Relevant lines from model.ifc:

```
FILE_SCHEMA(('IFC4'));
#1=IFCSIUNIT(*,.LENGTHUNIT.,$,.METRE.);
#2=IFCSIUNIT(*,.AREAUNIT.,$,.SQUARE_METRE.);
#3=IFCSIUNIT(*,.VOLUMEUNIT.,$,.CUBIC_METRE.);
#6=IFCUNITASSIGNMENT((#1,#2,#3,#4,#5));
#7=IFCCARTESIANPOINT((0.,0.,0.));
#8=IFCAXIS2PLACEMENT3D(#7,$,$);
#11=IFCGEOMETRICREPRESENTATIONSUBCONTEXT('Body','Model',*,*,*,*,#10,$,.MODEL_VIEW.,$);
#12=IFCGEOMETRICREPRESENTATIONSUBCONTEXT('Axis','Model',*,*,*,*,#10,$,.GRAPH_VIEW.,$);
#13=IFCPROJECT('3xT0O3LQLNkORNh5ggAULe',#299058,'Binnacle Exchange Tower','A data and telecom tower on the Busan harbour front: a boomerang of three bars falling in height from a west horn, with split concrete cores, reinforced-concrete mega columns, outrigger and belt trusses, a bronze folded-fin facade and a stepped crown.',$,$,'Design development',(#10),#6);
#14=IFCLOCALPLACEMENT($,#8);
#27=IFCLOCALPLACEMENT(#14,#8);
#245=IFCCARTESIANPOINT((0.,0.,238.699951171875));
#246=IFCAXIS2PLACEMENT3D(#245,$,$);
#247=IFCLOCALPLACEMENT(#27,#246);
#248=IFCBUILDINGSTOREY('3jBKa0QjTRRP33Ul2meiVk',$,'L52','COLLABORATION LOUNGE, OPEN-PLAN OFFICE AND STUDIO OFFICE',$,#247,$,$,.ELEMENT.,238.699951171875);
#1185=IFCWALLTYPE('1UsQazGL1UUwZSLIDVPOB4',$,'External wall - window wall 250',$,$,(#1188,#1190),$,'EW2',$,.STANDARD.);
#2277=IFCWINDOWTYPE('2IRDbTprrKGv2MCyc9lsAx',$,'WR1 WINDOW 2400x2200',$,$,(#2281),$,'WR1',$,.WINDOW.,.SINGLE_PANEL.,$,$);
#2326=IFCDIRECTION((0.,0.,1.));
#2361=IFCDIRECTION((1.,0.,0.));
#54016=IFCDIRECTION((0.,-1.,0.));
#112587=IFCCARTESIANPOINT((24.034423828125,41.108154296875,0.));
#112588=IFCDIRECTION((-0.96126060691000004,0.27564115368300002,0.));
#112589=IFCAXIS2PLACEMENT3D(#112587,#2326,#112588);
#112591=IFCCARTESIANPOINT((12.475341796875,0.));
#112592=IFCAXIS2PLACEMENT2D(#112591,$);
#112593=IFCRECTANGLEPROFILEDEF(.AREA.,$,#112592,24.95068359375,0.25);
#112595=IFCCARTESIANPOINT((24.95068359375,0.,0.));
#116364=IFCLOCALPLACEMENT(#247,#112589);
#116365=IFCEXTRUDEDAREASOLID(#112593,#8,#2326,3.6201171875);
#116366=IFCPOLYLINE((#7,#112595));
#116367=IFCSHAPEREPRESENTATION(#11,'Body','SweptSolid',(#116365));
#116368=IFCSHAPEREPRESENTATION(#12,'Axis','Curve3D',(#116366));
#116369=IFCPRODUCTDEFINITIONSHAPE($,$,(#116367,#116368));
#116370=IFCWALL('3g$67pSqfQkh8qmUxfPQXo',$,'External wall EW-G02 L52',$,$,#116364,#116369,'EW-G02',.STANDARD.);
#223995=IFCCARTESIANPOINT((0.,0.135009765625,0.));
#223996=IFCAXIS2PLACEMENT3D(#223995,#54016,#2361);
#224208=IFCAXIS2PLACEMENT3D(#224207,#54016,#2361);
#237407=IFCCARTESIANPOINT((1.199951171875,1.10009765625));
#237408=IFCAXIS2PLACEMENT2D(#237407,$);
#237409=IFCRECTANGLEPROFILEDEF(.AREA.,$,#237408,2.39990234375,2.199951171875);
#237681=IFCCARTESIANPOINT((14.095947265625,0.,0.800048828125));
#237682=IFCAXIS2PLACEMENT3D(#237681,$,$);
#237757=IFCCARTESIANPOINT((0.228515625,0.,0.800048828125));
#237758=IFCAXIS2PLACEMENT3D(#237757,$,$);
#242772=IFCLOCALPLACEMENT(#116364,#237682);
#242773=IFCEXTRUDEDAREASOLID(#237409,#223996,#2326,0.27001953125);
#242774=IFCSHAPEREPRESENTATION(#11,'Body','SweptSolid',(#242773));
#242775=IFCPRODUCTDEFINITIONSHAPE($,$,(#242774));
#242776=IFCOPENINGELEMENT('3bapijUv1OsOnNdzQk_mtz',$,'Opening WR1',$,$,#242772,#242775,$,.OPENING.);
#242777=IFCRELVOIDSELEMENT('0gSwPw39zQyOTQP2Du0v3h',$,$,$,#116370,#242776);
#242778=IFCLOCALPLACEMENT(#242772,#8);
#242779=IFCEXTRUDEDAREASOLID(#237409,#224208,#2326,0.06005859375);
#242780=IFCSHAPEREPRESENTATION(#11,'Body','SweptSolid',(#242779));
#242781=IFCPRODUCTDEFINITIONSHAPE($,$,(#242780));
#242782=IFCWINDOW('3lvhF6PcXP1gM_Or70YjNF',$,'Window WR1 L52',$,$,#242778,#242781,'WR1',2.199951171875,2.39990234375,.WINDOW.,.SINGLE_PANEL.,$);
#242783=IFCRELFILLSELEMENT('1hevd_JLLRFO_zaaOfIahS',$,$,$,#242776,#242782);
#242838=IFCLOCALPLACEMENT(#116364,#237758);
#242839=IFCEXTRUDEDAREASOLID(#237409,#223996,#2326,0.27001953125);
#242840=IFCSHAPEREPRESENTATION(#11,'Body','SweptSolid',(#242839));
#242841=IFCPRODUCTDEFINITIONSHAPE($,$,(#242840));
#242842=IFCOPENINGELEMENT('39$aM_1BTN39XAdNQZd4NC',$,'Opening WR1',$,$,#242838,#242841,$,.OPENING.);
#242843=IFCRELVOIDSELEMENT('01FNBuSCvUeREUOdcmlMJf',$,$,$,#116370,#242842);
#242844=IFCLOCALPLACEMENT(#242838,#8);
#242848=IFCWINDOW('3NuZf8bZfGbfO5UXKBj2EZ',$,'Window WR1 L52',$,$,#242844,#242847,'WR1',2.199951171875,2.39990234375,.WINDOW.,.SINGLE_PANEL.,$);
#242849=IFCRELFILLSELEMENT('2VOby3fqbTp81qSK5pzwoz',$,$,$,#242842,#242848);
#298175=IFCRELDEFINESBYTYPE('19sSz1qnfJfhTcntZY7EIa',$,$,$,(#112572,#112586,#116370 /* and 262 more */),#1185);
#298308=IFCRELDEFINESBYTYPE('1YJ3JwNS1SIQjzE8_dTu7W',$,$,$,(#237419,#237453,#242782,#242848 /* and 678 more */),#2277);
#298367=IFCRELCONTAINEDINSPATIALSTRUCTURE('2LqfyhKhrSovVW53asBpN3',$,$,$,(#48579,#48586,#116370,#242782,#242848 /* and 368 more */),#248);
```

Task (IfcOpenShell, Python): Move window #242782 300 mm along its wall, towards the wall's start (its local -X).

```python
import ifcopenshell
import ifcopenshell.api.geometry
import ifcopenshell.util.placement

model = ifcopenshell.open("model.ifc")

window = model.by_guid("3lvhF6PcXP1gM_Or70YjNF")
opening = window.FillsVoids[0].RelatingOpeningElement
wall = opening.VoidsElements[0].RelatingBuildingElement

wall_matrix = ifcopenshell.util.placement.get_local_placement(wall.ObjectPlacement)
shift = wall_matrix[:3, 0] * -0.3
before = ifcopenshell.util.placement.get_local_placement(window.ObjectPlacement)[:3, 3].copy()

# The window is placed relative to its opening, so it follows when the opening moves.
matrix = ifcopenshell.util.placement.get_local_placement(opening.ObjectPlacement)
matrix[:3, 3] += shift
ifcopenshell.api.geometry.edit_object_placement(
    model, product=opening, matrix=matrix, is_si=False, should_transform_children=True
)

after = ifcopenshell.util.placement.get_local_placement(window.ObjectPlacement)[:3, 3]
print("window moved by", (after - before).round(3) + 0.0)

model.write("model-out.ifc")
```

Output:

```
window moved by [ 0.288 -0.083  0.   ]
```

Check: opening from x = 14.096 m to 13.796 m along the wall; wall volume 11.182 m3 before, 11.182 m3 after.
